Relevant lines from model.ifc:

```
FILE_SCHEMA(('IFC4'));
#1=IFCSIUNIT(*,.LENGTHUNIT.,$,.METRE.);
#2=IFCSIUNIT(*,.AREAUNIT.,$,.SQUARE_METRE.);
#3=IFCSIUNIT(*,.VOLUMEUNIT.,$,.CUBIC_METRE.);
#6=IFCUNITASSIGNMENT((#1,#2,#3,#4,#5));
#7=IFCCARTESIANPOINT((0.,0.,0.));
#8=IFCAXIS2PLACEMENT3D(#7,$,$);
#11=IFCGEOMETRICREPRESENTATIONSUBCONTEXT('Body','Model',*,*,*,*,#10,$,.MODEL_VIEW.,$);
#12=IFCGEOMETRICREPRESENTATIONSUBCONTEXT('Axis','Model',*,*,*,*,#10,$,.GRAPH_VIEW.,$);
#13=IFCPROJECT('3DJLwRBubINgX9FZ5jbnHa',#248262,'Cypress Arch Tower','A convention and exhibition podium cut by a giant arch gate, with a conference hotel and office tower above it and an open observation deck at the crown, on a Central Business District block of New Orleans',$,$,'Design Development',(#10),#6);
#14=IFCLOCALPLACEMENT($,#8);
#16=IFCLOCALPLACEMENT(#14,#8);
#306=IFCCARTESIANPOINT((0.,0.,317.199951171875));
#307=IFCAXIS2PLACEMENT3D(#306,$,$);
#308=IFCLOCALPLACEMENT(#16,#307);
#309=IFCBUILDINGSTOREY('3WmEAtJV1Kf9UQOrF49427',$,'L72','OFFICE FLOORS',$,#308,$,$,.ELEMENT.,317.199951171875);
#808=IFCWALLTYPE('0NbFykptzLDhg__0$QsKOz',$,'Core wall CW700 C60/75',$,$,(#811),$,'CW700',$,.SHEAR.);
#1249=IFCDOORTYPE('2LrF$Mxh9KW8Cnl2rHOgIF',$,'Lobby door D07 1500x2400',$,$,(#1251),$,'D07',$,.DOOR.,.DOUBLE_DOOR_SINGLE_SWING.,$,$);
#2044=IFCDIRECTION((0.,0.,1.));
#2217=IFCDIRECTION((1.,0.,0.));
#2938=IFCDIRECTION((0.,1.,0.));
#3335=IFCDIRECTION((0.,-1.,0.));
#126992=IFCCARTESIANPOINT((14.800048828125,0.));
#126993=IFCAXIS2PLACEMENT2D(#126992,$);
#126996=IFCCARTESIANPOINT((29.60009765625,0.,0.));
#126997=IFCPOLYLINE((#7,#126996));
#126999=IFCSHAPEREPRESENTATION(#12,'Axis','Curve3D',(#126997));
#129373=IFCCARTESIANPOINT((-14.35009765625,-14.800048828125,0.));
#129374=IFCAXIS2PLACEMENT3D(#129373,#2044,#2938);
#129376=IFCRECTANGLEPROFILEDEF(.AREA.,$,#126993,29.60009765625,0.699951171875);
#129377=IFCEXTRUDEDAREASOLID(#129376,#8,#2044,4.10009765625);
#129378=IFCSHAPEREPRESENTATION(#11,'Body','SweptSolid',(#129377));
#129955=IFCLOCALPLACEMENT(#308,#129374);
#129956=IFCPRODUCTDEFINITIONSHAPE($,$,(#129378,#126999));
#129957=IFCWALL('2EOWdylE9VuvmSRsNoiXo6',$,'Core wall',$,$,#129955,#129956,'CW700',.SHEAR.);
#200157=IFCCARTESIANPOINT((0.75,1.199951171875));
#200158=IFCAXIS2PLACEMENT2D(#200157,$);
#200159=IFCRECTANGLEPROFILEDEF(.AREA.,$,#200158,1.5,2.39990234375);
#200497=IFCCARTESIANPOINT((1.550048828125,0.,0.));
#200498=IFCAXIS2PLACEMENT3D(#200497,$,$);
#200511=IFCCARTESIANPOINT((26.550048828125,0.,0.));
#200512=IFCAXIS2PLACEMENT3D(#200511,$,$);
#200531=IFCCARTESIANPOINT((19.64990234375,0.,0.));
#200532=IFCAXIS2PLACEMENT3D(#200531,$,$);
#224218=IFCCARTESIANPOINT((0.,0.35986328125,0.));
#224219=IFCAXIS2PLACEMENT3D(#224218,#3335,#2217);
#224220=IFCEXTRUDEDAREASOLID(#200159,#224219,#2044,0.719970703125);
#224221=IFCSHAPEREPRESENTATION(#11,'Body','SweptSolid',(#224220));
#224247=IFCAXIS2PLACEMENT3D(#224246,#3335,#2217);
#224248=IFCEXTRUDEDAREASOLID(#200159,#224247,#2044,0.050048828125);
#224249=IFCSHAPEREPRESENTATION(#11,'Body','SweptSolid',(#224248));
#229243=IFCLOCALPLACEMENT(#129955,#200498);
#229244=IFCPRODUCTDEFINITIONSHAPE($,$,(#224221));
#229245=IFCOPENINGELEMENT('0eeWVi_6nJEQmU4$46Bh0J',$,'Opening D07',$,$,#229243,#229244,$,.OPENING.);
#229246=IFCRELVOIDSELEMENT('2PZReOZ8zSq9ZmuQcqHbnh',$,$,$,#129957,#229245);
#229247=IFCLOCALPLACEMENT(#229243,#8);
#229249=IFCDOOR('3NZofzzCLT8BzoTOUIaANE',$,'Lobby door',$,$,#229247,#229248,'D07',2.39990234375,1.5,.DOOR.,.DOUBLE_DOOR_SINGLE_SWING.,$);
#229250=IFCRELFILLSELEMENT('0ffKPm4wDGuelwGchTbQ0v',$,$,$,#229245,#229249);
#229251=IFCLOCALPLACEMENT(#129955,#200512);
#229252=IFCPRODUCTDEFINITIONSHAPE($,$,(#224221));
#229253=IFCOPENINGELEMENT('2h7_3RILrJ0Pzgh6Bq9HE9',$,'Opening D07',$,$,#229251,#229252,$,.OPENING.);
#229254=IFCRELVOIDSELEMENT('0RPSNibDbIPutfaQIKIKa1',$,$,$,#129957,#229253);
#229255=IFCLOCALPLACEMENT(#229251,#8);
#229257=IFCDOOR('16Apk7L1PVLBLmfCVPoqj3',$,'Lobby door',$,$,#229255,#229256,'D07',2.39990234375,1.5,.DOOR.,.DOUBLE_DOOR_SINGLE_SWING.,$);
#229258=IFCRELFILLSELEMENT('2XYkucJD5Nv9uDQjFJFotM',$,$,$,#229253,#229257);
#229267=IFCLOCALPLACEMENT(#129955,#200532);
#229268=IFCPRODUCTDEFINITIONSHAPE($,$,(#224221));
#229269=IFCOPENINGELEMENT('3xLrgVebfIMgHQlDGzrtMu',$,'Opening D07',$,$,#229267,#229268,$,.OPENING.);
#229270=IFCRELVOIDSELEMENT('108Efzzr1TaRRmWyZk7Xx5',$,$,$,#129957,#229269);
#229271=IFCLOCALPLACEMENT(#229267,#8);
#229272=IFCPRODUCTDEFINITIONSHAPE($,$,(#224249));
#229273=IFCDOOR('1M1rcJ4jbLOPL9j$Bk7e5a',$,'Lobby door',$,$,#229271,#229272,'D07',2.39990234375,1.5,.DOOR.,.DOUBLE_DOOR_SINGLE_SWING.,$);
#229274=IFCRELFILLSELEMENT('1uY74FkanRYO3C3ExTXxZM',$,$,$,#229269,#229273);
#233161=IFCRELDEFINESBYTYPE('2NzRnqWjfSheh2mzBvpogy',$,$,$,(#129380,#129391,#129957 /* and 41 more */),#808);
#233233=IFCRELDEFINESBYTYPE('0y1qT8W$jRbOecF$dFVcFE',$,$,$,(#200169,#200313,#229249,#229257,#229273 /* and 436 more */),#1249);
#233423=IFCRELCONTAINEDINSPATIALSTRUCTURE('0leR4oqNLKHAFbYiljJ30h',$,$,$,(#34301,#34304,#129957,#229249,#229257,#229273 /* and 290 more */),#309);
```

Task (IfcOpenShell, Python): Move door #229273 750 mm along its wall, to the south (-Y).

```python
import ifcopenshell
import ifcopenshell.api.geometry
import ifcopenshell.util.placement
import ifcopenshell.util.unit

model = ifcopenshell.open("model.ifc")
unit_scale = ifcopenshell.util.unit.calculate_unit_scale(model)

door = model.by_guid("1M1rcJ4jbLOPL9j$Bk7e5a")
opening = door.FillsVoids[0].RelatingOpeningElement
wall = opening.VoidsElements[0].RelatingBuildingElement

wall_matrix = ifcopenshell.util.placement.get_local_placement(wall.ObjectPlacement)
shift = wall_matrix[:3, 0] * -0.75 / unit_scale
before = ifcopenshell.util.placement.get_local_placement(door.ObjectPlacement)[:3, 3].copy()

# The door is placed relative to its opening, so it follows when the opening moves.
matrix = ifcopenshell.util.placement.get_local_placement(opening.ObjectPlacement)
matrix[:3, 3] += shift
ifcopenshell.api.geometry.edit_object_placement(
    model, product=opening, matrix=matrix, is_si=False, should_transform_children=True
)

after = ifcopenshell.util.placement.get_local_placement(door.ObjectPlacement)[:3, 3]
print("door moved by", (after - before).round(3) + 0.0)

model.write("model_edited.ifc")
```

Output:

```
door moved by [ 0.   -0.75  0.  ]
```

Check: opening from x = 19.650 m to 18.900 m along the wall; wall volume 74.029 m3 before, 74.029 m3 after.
